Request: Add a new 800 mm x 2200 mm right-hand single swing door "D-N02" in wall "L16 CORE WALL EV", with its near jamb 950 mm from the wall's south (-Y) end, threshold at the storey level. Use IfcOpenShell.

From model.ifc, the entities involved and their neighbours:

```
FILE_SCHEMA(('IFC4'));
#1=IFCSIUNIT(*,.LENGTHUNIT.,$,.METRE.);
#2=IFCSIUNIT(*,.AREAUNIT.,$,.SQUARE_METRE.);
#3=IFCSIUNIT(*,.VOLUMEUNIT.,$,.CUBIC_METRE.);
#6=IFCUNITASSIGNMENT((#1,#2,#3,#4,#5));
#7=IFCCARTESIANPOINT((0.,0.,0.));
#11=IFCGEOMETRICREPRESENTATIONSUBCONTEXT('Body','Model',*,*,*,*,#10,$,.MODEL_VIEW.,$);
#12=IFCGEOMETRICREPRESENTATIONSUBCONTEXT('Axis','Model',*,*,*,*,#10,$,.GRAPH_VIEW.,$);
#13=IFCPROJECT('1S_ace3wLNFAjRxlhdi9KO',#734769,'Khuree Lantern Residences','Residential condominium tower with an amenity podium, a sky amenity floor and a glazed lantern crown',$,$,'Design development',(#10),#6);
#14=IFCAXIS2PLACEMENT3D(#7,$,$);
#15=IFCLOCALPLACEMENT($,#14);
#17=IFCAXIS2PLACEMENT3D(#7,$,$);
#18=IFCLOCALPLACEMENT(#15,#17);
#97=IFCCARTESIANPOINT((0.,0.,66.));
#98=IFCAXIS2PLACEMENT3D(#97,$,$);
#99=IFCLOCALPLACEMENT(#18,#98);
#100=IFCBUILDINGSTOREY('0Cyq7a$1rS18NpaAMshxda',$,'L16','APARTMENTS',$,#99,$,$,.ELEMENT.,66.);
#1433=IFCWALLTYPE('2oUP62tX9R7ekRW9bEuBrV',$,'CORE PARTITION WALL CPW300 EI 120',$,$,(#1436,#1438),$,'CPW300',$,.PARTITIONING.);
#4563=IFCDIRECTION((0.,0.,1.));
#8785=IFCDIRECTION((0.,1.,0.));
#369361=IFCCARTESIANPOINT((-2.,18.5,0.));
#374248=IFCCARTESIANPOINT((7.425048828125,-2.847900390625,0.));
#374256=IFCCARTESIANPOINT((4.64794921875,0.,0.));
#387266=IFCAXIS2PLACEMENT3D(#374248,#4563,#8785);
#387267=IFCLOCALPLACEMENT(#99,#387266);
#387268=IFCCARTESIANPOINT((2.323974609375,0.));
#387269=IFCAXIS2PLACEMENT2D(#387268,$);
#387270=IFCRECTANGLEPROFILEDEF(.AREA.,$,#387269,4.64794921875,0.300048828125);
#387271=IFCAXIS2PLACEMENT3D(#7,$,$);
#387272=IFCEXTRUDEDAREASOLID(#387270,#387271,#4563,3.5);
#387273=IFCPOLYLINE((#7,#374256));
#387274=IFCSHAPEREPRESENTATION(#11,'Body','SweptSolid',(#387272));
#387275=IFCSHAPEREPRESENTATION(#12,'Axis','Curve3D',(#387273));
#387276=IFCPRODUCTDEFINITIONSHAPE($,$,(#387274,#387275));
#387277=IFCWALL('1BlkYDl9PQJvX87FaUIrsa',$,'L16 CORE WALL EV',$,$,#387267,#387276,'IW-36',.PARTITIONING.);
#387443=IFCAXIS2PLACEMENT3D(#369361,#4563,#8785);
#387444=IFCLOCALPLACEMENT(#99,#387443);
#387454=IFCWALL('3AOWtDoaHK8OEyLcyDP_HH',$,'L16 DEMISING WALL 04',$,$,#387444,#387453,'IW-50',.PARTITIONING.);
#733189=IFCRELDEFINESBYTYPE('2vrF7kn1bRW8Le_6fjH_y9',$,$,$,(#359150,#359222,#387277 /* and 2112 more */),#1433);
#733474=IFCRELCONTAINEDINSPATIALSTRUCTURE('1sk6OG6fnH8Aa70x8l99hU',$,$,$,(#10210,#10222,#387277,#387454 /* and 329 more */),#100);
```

```python
import numpy as np
import ifcopenshell
import ifcopenshell.api.feature
import ifcopenshell.api.geometry
import ifcopenshell.api.root
import ifcopenshell.api.spatial
import ifcopenshell.geom
import ifcopenshell.util.element
import ifcopenshell.util.placement
import ifcopenshell.util.representation
import ifcopenshell.util.shape
import ifcopenshell.util.unit

model = ifcopenshell.open("model.ifc")
unit_scale = ifcopenshell.util.unit.calculate_unit_scale(model)
settings = ifcopenshell.geom.settings()


def volume(element):
    """Net volume in cubic metres, openings subtracted."""
    shape = ifcopenshell.geom.create_shape(settings, element)
    return ifcopenshell.util.shape.get_volume(shape.geometry)


wall = model.by_id(387277)
storey = ifcopenshell.util.element.get_container(wall, ifc_class="IfcBuildingStorey")
context = ifcopenshell.util.representation.get_context(model, "Model", "Body", "MODEL_VIEW")
before = volume(wall)

width, height, from_end, sill = 0.8, 2.2, 0.95, 0.0  # metres

# The wall runs along its own X axis, and the end named is its -X end.
wall_shape = ifcopenshell.geom.create_shape(settings, wall)
x, y, z = ifcopenshell.util.shape.get_vertices(wall_shape.geometry).T
start = x.min() + from_end
face, thickness = float(y.min()), float(y.max() - y.min())
wall_matrix = ifcopenshell.util.placement.get_local_placement(wall.ObjectPlacement)
level = ifcopenshell.util.placement.get_local_placement(storey.ObjectPlacement)[2, 3]


def in_wall(x, y):
    """Placement at x, y metres in the wall's axes, at sill height."""
    matrix = wall_matrix.copy()
    matrix[:, 3] = wall_matrix @ np.array([x / unit_scale, y / unit_scale, 0.0, 1.0])
    matrix[2, 3] = level + sill / unit_scale
    return matrix


# Opening: a box that overshoots both wall faces by 50 mm.
opening = ifcopenshell.api.root.create_entity(model, ifc_class="IfcOpeningElement", predefined_type="OPENING")
box = ifcopenshell.api.geometry.add_wall_representation(
    model, context=context, length=width, height=height, thickness=thickness + 0.1
)
ifcopenshell.api.geometry.assign_representation(model, product=opening, representation=box)
ifcopenshell.api.geometry.edit_object_placement(model, product=opening, matrix=in_wall(start, face - 0.05), is_si=False)
ifcopenshell.api.feature.add_feature(model, feature=opening, element=wall)

door = ifcopenshell.api.root.create_entity(model, ifc_class="IfcDoor", name="D-N02", predefined_type="DOOR")
door.OverallWidth, door.OverallHeight = width / unit_scale, height / unit_scale
door.OperationType = "SINGLE_SWING_RIGHT"
body = ifcopenshell.api.geometry.add_door_representation(
    model,
    context=context,
    overall_width=door.OverallWidth,
    overall_height=door.OverallHeight,
    operation_type="SINGLE_SWING_RIGHT",
    lining_properties={"LiningDepth": thickness / unit_scale, "ThresholdDepth": thickness / unit_scale},
)
ifcopenshell.api.geometry.assign_representation(model, product=door, representation=body)
ifcopenshell.api.spatial.assign_container(model, products=[door], relating_structure=storey)
ifcopenshell.api.feature.add_filling(model, opening=opening, element=door)

# The lining spans the wall, so the door starts at the wall face.
ifcopenshell.api.geometry.edit_object_placement(model, product=door, matrix=in_wall(start, face), is_si=False)

after = volume(wall)

print(f"wall volume {before:.3f} -> {after:.3f} m3")

model.write("model_edited.ifc")
```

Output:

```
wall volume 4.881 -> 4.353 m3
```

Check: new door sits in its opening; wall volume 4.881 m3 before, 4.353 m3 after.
